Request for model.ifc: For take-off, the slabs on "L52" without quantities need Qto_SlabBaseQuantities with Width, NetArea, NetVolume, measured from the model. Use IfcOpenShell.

First a look at what the model holds.

```python
import ifcopenshell
import ifcopenshell.util.element
import ifcopenshell.util.unit

model = ifcopenshell.open("model.ifc")
print(model.schema)
for unit_type in ("LENGTHUNIT", "AREAUNIT", "VOLUMEUNIT"):
    print(unit_type, ifcopenshell.util.unit.calculate_unit_scale(model, unit_type))
storey = next(s for s in model.by_type("IfcBuildingStorey") if s.Name == "L52")
slabs = [e for e in ifcopenshell.util.element.get_decomposition(storey) if e.is_a("IfcSlab")]
for e in sorted(slabs, key=lambda e: e.id()):
    print(e.id(), e.is_a(), e.Name, list(ifcopenshell.util.element.get_psets(e, qtos_only=True)), sep=" | ")
```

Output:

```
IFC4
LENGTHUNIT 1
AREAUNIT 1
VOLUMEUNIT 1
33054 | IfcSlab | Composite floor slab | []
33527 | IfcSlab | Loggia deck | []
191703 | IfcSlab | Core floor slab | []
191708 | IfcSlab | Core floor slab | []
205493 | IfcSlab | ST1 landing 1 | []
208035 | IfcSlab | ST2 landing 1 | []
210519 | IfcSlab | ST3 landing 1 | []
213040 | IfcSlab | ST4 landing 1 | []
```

```python
import ifcopenshell
import ifcopenshell.api.pset
import ifcopenshell.geom
import ifcopenshell.util.element
import ifcopenshell.util.shape
import ifcopenshell.util.unit

model = ifcopenshell.open("model.ifc")
unit_scale = ifcopenshell.util.unit.calculate_unit_scale(model)
area_scale = ifcopenshell.util.unit.calculate_unit_scale(model, "AREAUNIT")
volume_scale = ifcopenshell.util.unit.calculate_unit_scale(model, "VOLUMEUNIT")
settings = ifcopenshell.geom.settings()

storey = next(s for s in model.by_type("IfcBuildingStorey") if s.Name == "L52")
slabs = [e for e in ifcopenshell.util.element.get_decomposition(storey) if e.is_a("IfcSlab")]

for e in sorted(slabs, key=lambda e: e.id()):
    if ifcopenshell.util.element.get_psets(e, qtos_only=True, should_inherit=False):
        continue
    # Geometry comes back in metres, in the element's own axes.
    shape = ifcopenshell.geom.create_shape(settings, e)
    values = {
        "Width": ifcopenshell.util.shape.get_z(shape.geometry) / unit_scale,
        "NetArea": ifcopenshell.util.shape.get_footprint_area(shape.geometry) / area_scale,
        "NetVolume": ifcopenshell.util.shape.get_volume(shape.geometry) / volume_scale,
    }
    qto = ifcopenshell.api.pset.add_qto(model, product=e, name="Qto_SlabBaseQuantities")
    ifcopenshell.api.pset.edit_qto(model, qto=qto, properties=values)
    print(e.id(), {k: round(v, 3) for k, v in values.items()})

model.write("model_rev.ifc")
```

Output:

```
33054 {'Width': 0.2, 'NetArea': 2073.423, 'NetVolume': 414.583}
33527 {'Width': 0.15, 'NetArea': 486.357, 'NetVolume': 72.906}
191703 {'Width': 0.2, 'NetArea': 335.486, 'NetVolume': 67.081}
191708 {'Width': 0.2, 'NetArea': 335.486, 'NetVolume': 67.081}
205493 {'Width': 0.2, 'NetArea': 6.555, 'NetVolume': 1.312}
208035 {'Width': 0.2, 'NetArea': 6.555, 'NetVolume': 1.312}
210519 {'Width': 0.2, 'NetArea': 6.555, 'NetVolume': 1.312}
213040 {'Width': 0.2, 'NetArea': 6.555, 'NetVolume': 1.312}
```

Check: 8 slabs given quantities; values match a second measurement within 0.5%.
